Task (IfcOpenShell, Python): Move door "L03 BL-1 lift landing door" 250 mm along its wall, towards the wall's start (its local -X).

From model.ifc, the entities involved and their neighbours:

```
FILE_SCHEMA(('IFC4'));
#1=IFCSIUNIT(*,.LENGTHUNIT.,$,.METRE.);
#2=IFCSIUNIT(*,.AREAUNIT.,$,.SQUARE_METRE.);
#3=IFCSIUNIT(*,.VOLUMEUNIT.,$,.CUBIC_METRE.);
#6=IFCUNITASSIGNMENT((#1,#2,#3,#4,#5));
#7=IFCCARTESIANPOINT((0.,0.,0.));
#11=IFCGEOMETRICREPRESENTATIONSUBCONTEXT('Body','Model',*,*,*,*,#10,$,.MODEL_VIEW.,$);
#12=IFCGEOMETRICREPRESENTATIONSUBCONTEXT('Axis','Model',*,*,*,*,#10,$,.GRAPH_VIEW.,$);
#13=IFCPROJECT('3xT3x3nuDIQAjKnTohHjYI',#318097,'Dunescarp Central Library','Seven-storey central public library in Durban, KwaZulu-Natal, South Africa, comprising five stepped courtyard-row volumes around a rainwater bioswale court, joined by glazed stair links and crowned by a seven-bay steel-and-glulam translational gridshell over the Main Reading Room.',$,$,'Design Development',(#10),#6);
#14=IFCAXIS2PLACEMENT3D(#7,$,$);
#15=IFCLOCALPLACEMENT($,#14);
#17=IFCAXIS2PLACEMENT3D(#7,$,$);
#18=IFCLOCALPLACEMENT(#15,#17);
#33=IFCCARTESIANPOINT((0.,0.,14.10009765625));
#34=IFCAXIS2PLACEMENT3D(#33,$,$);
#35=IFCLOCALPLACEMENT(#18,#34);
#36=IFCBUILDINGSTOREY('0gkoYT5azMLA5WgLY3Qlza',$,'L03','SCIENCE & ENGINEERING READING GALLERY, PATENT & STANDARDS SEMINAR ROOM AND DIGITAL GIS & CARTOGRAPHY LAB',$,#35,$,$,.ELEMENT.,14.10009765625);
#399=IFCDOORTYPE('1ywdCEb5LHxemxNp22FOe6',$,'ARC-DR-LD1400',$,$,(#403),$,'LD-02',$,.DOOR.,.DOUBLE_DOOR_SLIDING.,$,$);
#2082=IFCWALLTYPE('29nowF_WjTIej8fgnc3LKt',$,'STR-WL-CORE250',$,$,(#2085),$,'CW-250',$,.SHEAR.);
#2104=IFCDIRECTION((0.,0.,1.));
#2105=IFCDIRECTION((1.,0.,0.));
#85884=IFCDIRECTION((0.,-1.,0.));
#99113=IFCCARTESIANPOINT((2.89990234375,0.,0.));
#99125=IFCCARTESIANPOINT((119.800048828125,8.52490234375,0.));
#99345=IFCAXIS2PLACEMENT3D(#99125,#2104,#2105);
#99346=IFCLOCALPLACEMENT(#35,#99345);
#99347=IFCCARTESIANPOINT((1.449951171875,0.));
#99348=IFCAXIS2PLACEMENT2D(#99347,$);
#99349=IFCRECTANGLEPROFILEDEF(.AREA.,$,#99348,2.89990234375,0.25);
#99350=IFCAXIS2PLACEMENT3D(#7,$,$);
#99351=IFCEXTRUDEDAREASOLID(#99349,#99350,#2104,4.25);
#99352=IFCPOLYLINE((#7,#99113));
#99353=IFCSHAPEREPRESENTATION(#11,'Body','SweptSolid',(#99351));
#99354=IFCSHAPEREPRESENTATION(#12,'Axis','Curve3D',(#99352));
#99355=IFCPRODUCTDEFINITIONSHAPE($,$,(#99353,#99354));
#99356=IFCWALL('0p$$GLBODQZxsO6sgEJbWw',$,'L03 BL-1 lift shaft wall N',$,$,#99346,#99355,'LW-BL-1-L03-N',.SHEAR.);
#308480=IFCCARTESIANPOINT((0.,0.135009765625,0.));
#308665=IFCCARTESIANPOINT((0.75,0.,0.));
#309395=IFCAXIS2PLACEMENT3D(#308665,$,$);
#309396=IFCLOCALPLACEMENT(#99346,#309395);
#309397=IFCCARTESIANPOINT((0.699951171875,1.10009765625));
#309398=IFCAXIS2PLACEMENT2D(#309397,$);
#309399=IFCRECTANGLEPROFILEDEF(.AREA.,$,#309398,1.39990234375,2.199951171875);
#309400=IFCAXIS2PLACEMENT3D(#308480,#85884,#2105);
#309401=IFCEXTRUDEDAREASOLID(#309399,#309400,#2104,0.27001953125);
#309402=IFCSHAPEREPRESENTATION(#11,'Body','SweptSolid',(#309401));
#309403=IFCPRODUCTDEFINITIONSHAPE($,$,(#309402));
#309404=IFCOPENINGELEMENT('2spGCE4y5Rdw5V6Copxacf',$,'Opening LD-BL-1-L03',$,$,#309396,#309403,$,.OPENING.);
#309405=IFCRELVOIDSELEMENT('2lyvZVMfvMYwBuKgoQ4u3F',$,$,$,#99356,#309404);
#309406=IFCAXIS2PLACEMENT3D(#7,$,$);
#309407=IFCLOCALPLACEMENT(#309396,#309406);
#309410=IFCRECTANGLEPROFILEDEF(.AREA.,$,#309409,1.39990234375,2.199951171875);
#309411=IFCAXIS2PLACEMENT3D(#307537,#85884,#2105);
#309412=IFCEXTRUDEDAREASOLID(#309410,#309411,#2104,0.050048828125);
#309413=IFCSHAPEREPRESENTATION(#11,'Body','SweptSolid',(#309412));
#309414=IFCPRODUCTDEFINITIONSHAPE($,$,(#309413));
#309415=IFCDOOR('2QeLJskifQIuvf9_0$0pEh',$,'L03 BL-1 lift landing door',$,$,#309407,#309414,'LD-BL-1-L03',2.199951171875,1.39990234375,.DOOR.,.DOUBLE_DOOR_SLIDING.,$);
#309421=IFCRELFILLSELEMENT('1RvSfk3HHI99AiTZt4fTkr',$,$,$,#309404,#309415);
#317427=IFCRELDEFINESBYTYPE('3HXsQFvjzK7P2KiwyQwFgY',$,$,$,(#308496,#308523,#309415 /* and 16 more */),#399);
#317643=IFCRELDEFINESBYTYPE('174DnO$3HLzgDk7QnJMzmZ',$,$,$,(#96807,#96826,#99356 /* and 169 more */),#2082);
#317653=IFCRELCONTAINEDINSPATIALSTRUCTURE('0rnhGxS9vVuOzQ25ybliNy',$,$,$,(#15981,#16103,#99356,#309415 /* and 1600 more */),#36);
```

```python
import ifcopenshell
import ifcopenshell.api.geometry
import ifcopenshell.util.placement
import ifcopenshell.util.unit

model = ifcopenshell.open("model.ifc")
unit_scale = ifcopenshell.util.unit.calculate_unit_scale(model)

door = model.by_id(309415)
opening = door.FillsVoids[0].RelatingOpeningElement
wall = opening.VoidsElements[0].RelatingBuildingElement

wall_matrix = ifcopenshell.util.placement.get_local_placement(wall.ObjectPlacement)
shift = wall_matrix[:3, 0] * -0.25 / unit_scale
before = ifcopenshell.util.placement.get_local_placement(door.ObjectPlacement)[:3, 3].copy()

# The door is placed relative to its opening, so it follows when the opening moves.
matrix = ifcopenshell.util.placement.get_local_placement(opening.ObjectPlacement)
matrix[:3, 3] += shift
ifcopenshell.api.geometry.edit_object_placement(
    model, product=opening, matrix=matrix, is_si=False, should_transform_children=True
)

after = ifcopenshell.util.placement.get_local_placement(door.ObjectPlacement)[:3, 3]
print("door moved by", (after - before).round(3) + 0.0)

model.write("model-out.ifc")
```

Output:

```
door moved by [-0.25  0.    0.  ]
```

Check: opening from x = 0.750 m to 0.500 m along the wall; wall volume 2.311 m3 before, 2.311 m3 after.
